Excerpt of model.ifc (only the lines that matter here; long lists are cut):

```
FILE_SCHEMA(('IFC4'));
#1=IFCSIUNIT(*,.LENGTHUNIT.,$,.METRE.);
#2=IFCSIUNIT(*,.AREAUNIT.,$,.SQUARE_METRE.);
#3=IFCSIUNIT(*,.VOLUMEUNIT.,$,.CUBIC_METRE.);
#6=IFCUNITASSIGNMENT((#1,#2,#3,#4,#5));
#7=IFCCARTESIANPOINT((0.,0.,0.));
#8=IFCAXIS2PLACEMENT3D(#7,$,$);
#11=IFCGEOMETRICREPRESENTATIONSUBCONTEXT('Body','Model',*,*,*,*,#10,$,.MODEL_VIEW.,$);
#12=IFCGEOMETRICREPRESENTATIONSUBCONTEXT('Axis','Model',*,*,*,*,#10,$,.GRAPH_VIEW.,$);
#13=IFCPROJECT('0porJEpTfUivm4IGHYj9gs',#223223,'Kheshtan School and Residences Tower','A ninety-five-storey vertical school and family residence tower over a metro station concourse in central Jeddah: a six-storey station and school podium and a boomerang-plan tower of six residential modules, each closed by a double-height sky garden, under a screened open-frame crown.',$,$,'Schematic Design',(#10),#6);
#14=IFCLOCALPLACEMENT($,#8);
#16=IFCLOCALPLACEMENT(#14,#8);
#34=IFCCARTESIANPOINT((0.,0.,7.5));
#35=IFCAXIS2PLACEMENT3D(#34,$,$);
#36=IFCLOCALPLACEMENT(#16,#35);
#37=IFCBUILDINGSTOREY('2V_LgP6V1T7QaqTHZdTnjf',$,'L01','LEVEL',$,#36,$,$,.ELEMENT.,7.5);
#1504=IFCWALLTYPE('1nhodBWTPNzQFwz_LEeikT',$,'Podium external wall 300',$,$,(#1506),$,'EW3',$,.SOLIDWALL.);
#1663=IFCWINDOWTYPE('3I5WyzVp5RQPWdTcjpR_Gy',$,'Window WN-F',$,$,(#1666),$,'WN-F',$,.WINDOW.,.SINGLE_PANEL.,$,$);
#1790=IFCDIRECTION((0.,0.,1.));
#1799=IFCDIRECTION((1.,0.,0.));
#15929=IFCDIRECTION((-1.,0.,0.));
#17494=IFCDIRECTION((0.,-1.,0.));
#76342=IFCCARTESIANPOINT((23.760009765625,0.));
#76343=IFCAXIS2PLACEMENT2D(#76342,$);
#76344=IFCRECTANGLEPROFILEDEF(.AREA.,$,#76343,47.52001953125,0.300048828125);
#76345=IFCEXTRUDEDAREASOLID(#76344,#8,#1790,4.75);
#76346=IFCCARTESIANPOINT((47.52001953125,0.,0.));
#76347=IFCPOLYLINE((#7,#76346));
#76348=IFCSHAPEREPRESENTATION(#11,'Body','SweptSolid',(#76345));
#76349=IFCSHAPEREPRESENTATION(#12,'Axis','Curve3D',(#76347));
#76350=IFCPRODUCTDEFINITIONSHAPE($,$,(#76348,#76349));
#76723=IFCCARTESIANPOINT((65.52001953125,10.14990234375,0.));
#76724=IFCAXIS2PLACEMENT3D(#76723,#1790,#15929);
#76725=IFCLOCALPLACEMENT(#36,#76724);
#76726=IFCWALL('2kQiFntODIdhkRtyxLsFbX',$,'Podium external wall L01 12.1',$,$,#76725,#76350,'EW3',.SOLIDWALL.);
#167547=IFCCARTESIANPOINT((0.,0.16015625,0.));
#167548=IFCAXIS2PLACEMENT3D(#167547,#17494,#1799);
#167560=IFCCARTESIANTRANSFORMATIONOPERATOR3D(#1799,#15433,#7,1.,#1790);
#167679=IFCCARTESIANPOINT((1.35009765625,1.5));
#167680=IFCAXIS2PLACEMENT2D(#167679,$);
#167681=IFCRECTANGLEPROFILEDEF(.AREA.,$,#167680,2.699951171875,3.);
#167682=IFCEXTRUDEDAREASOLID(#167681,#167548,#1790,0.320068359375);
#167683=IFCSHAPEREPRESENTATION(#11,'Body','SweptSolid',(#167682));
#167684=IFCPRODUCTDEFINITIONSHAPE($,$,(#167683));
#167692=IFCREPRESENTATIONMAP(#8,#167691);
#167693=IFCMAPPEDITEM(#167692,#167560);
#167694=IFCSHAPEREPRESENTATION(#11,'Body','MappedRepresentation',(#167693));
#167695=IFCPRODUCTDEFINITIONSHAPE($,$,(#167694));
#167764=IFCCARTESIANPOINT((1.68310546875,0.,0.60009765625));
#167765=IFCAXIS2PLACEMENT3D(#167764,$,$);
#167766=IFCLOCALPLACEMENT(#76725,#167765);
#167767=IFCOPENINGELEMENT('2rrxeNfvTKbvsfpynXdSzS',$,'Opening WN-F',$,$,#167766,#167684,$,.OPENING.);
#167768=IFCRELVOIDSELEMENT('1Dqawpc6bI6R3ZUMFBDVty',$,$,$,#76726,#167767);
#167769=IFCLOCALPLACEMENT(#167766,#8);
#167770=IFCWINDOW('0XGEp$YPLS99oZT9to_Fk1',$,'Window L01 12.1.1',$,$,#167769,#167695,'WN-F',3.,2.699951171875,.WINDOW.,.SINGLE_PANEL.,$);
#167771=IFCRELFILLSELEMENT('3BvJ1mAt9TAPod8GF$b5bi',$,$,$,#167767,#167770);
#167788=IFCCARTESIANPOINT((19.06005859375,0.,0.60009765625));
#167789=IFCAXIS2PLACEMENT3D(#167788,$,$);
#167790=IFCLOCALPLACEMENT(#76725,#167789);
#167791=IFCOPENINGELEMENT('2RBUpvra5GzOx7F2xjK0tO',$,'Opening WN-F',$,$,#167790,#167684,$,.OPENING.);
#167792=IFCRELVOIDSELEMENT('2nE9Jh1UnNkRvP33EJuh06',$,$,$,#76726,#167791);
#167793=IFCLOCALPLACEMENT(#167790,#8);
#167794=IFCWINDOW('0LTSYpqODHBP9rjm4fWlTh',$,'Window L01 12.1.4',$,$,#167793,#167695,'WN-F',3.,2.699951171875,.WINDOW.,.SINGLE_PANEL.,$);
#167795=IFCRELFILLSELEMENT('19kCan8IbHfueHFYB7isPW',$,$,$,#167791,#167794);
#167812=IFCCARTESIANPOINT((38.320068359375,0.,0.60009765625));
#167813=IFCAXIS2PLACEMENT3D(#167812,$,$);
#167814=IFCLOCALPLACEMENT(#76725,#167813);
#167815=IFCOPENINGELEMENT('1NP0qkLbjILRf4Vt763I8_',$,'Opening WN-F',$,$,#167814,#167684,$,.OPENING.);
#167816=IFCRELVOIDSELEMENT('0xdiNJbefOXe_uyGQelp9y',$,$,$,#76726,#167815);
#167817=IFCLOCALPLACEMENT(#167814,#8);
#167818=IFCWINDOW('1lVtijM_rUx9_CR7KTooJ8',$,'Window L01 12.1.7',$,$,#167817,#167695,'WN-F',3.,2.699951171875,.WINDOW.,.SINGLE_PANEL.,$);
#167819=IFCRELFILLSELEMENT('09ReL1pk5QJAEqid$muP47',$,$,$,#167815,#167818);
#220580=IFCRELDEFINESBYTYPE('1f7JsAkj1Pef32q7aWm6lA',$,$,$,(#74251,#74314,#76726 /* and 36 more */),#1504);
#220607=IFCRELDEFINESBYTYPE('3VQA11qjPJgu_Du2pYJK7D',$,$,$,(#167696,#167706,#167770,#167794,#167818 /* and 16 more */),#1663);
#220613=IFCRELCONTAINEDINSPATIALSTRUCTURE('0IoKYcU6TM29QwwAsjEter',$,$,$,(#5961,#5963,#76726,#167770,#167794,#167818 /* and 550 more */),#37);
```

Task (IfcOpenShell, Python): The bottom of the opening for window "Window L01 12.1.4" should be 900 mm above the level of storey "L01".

```python
import numpy as np
import ifcopenshell
import ifcopenshell.api.geometry
import ifcopenshell.geom
import ifcopenshell.util.element
import ifcopenshell.util.placement
import ifcopenshell.util.shape
import ifcopenshell.util.unit

model = ifcopenshell.open("model.ifc")
unit_scale = ifcopenshell.util.unit.calculate_unit_scale(model)

window = model.by_guid("0LTSYpqODHBP9rjm4fWlTh")
opening = window.FillsVoids[0].RelatingOpeningElement
storey = ifcopenshell.util.element.get_container(window, ifc_class="IfcBuildingStorey")
level = ifcopenshell.util.placement.get_local_placement(storey.ObjectPlacement)[2, 3]

# The opening's origin need not be at the sill, so measure its lowest point.
shape = ifcopenshell.geom.create_shape(ifcopenshell.geom.settings(), opening)
bottom = ifcopenshell.util.shape.get_shape_bottom_elevation(shape, shape.geometry) / unit_scale
dz = level + 0.9 / unit_scale - bottom

shift = np.array([0.0, 0.0, dz])
# The window is placed relative to its opening, so it follows when the opening moves.
matrix = ifcopenshell.util.placement.get_local_placement(opening.ObjectPlacement)
matrix[:3, 3] += shift
ifcopenshell.api.geometry.edit_object_placement(
    model, product=opening, matrix=matrix, is_si=False, should_transform_children=True
)

print(f"moved by {dz * unit_scale:+.3f} m")

model.write("model_v2.ifc")
```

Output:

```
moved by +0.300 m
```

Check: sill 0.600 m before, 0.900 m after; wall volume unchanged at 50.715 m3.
